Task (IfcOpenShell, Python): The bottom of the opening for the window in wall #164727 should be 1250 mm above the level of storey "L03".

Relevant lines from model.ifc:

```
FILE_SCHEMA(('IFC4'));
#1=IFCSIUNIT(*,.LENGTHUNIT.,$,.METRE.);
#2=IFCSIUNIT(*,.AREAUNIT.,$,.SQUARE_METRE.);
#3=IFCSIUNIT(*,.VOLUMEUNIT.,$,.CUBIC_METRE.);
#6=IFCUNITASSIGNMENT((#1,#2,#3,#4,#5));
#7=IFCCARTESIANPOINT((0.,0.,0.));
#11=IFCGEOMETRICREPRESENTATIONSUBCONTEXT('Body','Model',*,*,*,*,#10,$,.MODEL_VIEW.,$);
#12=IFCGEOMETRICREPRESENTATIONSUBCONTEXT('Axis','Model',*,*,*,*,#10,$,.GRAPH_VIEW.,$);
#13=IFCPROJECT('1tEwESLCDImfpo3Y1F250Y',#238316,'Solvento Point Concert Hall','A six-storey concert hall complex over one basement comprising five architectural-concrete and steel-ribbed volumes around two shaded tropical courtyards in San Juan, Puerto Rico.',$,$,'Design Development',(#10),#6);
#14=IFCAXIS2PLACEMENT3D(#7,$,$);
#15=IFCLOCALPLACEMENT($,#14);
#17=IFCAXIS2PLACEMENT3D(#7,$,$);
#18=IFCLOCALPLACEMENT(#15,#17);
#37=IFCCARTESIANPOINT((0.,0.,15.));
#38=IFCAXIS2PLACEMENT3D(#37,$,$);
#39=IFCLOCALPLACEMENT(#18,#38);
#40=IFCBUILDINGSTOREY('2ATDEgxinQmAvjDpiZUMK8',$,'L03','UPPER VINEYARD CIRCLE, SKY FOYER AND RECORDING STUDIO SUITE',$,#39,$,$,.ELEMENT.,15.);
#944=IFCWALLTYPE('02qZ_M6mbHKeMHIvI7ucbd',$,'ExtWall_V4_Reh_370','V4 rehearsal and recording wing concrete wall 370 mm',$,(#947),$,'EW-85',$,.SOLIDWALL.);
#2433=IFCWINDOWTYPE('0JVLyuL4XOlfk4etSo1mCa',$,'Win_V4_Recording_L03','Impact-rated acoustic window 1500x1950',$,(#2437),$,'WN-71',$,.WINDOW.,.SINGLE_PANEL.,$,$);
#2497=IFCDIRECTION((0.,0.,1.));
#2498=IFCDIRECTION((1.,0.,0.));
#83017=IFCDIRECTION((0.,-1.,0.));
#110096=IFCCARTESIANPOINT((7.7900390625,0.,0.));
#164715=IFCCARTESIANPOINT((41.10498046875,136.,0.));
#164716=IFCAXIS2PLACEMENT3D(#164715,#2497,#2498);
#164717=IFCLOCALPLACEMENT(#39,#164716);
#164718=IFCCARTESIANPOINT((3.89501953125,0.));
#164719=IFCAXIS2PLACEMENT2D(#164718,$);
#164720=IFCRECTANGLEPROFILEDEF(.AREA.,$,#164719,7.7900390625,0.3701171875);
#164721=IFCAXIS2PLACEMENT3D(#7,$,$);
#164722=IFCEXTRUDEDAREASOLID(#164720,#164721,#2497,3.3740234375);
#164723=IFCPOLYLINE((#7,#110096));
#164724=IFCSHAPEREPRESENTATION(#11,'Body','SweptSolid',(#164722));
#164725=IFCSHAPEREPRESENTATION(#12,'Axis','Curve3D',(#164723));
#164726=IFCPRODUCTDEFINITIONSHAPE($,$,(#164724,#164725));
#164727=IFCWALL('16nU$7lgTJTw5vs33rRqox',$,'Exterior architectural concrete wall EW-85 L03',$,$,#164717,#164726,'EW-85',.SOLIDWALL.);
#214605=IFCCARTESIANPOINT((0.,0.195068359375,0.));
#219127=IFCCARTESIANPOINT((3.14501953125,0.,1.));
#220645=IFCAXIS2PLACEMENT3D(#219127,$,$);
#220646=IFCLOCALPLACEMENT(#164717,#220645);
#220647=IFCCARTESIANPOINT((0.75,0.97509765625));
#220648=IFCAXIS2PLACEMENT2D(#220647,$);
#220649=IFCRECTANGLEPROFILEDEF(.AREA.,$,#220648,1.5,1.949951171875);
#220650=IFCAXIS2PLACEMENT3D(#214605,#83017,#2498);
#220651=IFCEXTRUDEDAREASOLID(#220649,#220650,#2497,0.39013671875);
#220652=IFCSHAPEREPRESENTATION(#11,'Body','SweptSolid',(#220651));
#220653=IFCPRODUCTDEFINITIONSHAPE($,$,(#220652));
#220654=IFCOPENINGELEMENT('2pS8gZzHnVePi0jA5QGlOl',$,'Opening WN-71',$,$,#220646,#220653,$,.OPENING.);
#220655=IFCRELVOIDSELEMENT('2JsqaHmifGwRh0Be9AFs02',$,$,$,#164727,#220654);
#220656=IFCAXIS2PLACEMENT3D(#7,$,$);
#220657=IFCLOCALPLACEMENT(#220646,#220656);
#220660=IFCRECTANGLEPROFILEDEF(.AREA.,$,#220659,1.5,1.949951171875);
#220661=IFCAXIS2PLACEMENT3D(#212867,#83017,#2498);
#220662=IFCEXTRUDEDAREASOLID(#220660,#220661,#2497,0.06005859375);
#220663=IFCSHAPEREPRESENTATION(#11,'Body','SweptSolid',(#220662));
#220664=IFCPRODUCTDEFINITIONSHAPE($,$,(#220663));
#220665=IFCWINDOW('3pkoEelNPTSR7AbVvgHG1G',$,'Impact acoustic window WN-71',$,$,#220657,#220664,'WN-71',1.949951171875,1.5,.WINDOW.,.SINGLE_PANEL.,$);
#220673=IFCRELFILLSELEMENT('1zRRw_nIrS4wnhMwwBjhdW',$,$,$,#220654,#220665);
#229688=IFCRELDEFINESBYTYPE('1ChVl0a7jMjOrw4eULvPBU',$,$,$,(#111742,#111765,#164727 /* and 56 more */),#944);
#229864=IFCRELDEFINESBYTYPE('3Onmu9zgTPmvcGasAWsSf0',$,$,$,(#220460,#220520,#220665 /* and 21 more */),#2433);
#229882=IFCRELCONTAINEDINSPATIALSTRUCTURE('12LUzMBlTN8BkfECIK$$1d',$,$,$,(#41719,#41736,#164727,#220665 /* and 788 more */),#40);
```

```python
import numpy as np
import ifcopenshell
import ifcopenshell.api.geometry
import ifcopenshell.geom
import ifcopenshell.util.element
import ifcopenshell.util.placement
import ifcopenshell.util.shape
import ifcopenshell.util.unit

model = ifcopenshell.open("model.ifc")
unit_scale = ifcopenshell.util.unit.calculate_unit_scale(model)

window = model.by_guid("3pkoEelNPTSR7AbVvgHG1G")
opening = window.FillsVoids[0].RelatingOpeningElement
storey = ifcopenshell.util.element.get_container(window, ifc_class="IfcBuildingStorey")
level = ifcopenshell.util.placement.get_local_placement(storey.ObjectPlacement)[2, 3]

# The opening's origin need not be at the sill, so measure its lowest point.
shape = ifcopenshell.geom.create_shape(ifcopenshell.geom.settings(), opening)
bottom = ifcopenshell.util.shape.get_shape_bottom_elevation(shape, shape.geometry) / unit_scale
dz = level + 1.25 - bottom

shift = np.array([0.0, 0.0, dz])
# The window is placed relative to its opening, so it follows when the opening moves.
matrix = ifcopenshell.util.placement.get_local_placement(opening.ObjectPlacement)
matrix[:3, 3] += shift
ifcopenshell.api.geometry.edit_object_placement(
    model, product=opening, matrix=matrix, is_si=False, should_transform_children=True
)

print(f"moved by {dz * unit_scale:+.3f} m")

model.write("model_rev.ifc")
```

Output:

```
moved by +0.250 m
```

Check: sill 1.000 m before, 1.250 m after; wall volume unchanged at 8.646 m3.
